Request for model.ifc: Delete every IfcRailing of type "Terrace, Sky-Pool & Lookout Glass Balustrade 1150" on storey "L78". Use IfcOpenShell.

First a look at what the model holds.

```python
import ifcopenshell
import ifcopenshell.util.element

model = ifcopenshell.open("model.ifc")
print(model.schema)
storey = next(s for s in model.by_type("IfcBuildingStorey") if s.Name == "L78")
railings = [e for e in ifcopenshell.util.element.get_decomposition(storey) if e.is_a("IfcRailing")]
seen = {}
for e in railings:
    element_type = ifcopenshell.util.element.get_type(e)
    name = element_type.Name if element_type not in (None, e) else None
    seen[name] = seen.get(name, 0) + 1
for name, count in sorted(seen.items(), key=str):
    print(count, "x", name)
```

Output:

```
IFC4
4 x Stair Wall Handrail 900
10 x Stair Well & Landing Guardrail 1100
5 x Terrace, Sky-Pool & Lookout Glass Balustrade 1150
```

```python
import ifcopenshell
import ifcopenshell.api.root
import ifcopenshell.util.element

model = ifcopenshell.open("model.ifc")

storey = next(s for s in model.by_type("IfcBuildingStorey") if s.Name == "L78")
railings = [e for e in ifcopenshell.util.element.get_decomposition(storey) if e.is_a("IfcRailing")]
targets = [e for e in railings if (t := ifcopenshell.util.element.get_type(e)) not in (None, e) and t.Name == "Terrace, Sky-Pool & Lookout Glass Balustrade 1150"]

for e in targets:
    ifcopenshell.api.root.remove_product(model, product=e)
print(len(targets), "removed")

model.write("model_edited.ifc")
```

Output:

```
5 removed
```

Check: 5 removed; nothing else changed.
